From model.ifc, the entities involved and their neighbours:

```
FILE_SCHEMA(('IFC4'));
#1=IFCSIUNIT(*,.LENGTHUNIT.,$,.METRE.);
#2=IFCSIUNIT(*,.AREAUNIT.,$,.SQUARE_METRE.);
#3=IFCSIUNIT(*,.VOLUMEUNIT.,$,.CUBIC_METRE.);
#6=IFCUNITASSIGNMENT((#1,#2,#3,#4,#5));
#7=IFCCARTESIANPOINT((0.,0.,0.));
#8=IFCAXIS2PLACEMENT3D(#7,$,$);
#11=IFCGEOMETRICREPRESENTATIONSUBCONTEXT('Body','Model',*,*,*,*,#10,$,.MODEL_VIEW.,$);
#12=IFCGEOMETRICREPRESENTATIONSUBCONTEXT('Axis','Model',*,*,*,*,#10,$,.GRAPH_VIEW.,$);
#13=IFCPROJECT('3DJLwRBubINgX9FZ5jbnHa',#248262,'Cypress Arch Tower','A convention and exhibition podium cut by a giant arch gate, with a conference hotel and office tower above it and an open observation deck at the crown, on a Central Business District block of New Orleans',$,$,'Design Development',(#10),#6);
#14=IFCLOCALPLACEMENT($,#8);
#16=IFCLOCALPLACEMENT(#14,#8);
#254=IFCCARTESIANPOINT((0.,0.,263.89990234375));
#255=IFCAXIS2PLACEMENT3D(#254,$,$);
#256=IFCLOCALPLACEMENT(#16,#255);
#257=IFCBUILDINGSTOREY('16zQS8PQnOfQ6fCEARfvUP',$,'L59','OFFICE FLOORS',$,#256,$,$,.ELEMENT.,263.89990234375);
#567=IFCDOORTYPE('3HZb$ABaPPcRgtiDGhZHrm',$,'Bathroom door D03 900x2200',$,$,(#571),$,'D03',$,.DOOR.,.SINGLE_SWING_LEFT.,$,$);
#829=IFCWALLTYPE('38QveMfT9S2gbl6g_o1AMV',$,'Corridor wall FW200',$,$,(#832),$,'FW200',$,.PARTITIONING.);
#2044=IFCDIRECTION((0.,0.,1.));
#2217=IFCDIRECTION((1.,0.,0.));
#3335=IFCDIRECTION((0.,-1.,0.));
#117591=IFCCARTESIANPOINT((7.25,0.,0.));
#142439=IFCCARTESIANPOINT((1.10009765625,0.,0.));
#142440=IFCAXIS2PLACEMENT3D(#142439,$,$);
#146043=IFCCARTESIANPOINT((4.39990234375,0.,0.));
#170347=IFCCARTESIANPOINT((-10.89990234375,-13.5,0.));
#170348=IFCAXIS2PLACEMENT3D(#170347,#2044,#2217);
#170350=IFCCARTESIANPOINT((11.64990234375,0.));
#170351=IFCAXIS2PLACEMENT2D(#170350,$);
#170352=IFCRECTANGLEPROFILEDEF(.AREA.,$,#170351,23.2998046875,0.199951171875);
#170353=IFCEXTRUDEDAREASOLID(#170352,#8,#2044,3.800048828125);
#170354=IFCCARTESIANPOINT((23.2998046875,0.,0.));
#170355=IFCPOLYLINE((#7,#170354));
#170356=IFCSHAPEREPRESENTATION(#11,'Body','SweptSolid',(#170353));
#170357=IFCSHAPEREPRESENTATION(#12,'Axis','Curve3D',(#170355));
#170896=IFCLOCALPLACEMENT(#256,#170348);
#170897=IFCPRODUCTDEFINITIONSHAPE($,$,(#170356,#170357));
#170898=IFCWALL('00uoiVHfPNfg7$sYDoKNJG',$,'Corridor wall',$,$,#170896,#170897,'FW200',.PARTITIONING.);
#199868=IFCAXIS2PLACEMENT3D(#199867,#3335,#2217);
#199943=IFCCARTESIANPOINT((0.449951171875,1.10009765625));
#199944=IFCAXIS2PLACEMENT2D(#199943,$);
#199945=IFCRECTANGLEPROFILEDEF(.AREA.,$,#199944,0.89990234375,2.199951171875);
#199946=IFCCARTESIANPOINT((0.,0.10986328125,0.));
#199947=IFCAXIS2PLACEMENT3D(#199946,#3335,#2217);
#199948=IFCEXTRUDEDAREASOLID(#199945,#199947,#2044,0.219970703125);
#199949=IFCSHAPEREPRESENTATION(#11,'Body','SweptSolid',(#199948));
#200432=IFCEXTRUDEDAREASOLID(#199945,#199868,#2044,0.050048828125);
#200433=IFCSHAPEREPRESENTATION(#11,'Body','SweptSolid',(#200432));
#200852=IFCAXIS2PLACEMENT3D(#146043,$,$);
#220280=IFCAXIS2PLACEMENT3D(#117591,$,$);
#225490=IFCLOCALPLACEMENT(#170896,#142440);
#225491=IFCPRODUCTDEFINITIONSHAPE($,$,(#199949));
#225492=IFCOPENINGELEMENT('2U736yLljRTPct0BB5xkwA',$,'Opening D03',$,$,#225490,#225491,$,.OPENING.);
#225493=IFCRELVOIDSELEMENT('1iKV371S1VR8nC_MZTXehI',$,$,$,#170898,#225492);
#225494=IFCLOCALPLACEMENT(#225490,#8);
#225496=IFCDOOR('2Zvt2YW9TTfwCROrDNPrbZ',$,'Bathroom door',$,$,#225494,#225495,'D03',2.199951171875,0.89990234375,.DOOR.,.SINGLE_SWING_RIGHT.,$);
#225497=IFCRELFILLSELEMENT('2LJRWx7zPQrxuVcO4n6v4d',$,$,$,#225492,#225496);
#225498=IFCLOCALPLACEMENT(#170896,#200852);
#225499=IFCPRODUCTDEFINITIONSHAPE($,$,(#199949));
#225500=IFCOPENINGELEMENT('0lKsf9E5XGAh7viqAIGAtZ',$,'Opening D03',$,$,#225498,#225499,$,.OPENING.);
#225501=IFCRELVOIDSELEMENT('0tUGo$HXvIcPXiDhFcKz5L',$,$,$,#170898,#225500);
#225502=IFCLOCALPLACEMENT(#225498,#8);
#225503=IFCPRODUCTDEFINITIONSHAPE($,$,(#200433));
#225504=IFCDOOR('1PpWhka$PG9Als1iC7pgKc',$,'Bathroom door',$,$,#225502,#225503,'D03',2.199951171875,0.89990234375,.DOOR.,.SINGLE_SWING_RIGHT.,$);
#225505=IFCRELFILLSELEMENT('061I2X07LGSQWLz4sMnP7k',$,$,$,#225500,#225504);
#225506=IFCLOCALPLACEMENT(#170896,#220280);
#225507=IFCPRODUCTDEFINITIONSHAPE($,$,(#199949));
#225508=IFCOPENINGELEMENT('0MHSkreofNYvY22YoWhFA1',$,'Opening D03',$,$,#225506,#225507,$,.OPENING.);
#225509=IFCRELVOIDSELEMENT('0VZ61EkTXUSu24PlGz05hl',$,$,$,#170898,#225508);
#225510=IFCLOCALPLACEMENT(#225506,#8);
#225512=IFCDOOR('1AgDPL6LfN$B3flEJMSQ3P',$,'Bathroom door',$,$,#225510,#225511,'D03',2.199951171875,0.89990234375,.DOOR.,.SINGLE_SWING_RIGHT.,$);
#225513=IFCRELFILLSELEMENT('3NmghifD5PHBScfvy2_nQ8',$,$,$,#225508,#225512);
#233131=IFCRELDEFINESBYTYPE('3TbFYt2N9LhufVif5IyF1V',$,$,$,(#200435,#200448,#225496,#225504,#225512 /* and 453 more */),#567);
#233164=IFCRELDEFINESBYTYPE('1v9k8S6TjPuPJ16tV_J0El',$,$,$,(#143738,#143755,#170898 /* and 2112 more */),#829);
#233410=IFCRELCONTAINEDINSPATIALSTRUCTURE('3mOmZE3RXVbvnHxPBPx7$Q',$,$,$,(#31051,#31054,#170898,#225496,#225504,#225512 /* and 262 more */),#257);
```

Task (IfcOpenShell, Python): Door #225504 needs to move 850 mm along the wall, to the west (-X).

```python
import ifcopenshell
import ifcopenshell.api.geometry
import ifcopenshell.util.placement
import ifcopenshell.util.unit

model = ifcopenshell.open("model.ifc")
unit_scale = ifcopenshell.util.unit.calculate_unit_scale(model)

door = model.by_guid("1PpWhka$PG9Als1iC7pgKc")
opening = door.FillsVoids[0].RelatingOpeningElement
wall = opening.VoidsElements[0].RelatingBuildingElement

wall_matrix = ifcopenshell.util.placement.get_local_placement(wall.ObjectPlacement)
shift = wall_matrix[:3, 0] * -0.85 / unit_scale
before = ifcopenshell.util.placement.get_local_placement(door.ObjectPlacement)[:3, 3].copy()

# The door is placed relative to its opening, so it follows when the opening moves.
matrix = ifcopenshell.util.placement.get_local_placement(opening.ObjectPlacement)
matrix[:3, 3] += shift
ifcopenshell.api.geometry.edit_object_placement(
    model, product=opening, matrix=matrix, is_si=False, should_transform_children=True
)

after = ifcopenshell.util.placement.get_local_placement(door.ObjectPlacement)[:3, 3]
print("door moved by", (after - before).round(3) + 0.0)

model.write("model_updated.ifc")
```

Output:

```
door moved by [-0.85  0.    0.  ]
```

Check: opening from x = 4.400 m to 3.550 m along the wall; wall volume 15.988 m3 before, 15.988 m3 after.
